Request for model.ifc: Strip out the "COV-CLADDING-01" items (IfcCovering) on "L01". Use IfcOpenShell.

First a look at what the model holds.

```python
import ifcopenshell
import ifcopenshell.util.element

model = ifcopenshell.open("model.ifc")
print(model.schema)
storey = next(s for s in model.by_type("IfcBuildingStorey") if s.Name == "L01")
coverings = [e for e in ifcopenshell.util.element.get_decomposition(storey) if e.is_a("IfcCovering")]
seen = {}
for e in coverings:
    element_type = ifcopenshell.util.element.get_type(e)
    name = element_type.Name if element_type not in (None, e) else None
    seen[name] = seen.get(name, 0) + 1
for name, count in sorted(seen.items(), key=str):
    print(count, "x", name)
```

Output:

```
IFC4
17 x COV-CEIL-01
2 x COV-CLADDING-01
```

```python
import ifcopenshell
import ifcopenshell.api.root
import ifcopenshell.util.element

model = ifcopenshell.open("model.ifc")

storey = next(s for s in model.by_type("IfcBuildingStorey") if s.Name == "L01")
coverings = [e for e in ifcopenshell.util.element.get_decomposition(storey) if e.is_a("IfcCovering")]
targets = [e for e in coverings if (t := ifcopenshell.util.element.get_type(e)) not in (None, e) and t.Name == "COV-CLADDING-01"]

for e in targets:
    ifcopenshell.api.root.remove_product(model, product=e)
print(len(targets), "removed")

model.write("model-out.ifc")
```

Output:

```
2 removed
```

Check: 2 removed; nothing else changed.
